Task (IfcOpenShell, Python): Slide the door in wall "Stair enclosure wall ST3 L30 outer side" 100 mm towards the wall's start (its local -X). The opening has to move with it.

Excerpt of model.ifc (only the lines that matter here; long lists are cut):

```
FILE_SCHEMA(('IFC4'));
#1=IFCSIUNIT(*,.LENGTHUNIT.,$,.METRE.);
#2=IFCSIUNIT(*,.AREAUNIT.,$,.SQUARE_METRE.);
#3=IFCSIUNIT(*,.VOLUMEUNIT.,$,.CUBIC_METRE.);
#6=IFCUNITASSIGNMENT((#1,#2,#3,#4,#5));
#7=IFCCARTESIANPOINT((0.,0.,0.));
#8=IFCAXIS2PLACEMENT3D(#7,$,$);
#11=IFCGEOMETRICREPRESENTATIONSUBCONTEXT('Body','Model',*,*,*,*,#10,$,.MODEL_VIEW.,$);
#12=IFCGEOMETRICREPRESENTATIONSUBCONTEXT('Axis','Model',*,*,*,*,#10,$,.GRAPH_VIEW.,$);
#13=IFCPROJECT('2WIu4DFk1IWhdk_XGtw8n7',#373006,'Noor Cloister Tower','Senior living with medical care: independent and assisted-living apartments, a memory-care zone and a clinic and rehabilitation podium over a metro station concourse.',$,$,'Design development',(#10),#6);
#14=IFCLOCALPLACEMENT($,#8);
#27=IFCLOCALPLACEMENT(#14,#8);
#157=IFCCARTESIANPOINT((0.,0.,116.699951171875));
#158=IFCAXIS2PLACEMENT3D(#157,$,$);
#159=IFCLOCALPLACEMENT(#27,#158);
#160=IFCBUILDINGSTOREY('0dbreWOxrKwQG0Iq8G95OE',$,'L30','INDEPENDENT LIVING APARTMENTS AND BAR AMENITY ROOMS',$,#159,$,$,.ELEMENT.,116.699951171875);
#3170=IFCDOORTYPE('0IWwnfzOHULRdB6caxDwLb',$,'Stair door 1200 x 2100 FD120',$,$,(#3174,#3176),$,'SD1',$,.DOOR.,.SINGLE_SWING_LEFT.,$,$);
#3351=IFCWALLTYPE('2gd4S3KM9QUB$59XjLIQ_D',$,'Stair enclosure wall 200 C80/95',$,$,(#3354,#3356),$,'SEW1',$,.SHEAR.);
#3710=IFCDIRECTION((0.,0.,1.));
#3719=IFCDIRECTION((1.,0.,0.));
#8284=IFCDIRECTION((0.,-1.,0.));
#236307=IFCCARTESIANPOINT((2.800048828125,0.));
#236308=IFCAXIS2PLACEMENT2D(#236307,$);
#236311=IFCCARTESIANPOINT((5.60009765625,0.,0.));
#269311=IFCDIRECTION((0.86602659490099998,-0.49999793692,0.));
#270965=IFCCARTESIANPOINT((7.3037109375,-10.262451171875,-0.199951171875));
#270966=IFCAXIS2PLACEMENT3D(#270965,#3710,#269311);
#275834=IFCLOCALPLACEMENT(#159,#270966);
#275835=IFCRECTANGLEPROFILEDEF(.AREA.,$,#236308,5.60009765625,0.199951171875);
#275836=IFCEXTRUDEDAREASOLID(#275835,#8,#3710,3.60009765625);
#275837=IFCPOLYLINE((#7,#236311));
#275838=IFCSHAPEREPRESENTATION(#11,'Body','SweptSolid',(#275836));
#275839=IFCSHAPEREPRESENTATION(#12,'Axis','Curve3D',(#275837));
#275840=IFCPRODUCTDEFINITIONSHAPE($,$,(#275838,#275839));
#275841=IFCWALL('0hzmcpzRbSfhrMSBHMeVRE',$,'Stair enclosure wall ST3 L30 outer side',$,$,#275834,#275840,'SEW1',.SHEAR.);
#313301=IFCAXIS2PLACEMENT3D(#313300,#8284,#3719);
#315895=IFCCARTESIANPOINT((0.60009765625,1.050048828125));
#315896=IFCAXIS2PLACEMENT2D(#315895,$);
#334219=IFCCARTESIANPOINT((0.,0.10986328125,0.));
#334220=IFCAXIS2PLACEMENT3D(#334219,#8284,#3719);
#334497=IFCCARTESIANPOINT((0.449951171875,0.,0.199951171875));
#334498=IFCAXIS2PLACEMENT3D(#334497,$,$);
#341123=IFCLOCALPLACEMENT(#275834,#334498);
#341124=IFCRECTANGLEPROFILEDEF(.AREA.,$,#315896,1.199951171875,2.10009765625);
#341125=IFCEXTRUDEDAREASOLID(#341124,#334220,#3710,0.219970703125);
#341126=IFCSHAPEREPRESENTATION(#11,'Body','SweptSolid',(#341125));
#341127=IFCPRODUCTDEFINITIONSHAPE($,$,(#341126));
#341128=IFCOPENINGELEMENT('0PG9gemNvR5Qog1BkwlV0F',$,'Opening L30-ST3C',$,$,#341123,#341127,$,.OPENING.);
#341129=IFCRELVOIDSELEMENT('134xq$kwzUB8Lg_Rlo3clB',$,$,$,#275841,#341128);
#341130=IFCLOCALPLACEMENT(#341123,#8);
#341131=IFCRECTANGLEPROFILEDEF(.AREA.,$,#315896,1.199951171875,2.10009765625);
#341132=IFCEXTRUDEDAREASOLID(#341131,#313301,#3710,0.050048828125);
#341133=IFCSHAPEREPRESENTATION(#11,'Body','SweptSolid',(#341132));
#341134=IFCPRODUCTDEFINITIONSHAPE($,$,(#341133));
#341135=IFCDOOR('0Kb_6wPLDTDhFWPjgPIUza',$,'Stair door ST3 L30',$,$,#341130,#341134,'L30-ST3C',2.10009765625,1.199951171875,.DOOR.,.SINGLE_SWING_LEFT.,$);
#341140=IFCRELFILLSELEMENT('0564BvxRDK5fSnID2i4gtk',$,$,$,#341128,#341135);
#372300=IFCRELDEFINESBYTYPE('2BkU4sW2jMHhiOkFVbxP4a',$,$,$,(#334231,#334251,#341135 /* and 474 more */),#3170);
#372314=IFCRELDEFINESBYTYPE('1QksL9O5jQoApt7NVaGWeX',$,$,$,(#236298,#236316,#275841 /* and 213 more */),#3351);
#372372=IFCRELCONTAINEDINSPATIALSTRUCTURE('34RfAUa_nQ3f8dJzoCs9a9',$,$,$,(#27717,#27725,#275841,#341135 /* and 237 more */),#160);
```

```python
import ifcopenshell
import ifcopenshell.api.geometry
import ifcopenshell.util.placement
import ifcopenshell.util.unit

model = ifcopenshell.open("model.ifc")
unit_scale = ifcopenshell.util.unit.calculate_unit_scale(model)

door = model.by_id(341135)
opening = door.FillsVoids[0].RelatingOpeningElement
wall = opening.VoidsElements[0].RelatingBuildingElement

wall_matrix = ifcopenshell.util.placement.get_local_placement(wall.ObjectPlacement)
shift = wall_matrix[:3, 0] * -0.1 / unit_scale
before = ifcopenshell.util.placement.get_local_placement(door.ObjectPlacement)[:3, 3].copy()

# The door is placed relative to its opening, so it follows when the opening moves.
matrix = ifcopenshell.util.placement.get_local_placement(opening.ObjectPlacement)
matrix[:3, 3] += shift
ifcopenshell.api.geometry.edit_object_placement(
    model, product=opening, matrix=matrix, is_si=False, should_transform_children=True
)

after = ifcopenshell.util.placement.get_local_placement(door.ObjectPlacement)[:3, 3]
print("door moved by", (after - before).round(3) + 0.0)

model.write("model_v2.ifc")
```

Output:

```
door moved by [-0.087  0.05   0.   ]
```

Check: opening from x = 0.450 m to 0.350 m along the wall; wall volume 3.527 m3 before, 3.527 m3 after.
